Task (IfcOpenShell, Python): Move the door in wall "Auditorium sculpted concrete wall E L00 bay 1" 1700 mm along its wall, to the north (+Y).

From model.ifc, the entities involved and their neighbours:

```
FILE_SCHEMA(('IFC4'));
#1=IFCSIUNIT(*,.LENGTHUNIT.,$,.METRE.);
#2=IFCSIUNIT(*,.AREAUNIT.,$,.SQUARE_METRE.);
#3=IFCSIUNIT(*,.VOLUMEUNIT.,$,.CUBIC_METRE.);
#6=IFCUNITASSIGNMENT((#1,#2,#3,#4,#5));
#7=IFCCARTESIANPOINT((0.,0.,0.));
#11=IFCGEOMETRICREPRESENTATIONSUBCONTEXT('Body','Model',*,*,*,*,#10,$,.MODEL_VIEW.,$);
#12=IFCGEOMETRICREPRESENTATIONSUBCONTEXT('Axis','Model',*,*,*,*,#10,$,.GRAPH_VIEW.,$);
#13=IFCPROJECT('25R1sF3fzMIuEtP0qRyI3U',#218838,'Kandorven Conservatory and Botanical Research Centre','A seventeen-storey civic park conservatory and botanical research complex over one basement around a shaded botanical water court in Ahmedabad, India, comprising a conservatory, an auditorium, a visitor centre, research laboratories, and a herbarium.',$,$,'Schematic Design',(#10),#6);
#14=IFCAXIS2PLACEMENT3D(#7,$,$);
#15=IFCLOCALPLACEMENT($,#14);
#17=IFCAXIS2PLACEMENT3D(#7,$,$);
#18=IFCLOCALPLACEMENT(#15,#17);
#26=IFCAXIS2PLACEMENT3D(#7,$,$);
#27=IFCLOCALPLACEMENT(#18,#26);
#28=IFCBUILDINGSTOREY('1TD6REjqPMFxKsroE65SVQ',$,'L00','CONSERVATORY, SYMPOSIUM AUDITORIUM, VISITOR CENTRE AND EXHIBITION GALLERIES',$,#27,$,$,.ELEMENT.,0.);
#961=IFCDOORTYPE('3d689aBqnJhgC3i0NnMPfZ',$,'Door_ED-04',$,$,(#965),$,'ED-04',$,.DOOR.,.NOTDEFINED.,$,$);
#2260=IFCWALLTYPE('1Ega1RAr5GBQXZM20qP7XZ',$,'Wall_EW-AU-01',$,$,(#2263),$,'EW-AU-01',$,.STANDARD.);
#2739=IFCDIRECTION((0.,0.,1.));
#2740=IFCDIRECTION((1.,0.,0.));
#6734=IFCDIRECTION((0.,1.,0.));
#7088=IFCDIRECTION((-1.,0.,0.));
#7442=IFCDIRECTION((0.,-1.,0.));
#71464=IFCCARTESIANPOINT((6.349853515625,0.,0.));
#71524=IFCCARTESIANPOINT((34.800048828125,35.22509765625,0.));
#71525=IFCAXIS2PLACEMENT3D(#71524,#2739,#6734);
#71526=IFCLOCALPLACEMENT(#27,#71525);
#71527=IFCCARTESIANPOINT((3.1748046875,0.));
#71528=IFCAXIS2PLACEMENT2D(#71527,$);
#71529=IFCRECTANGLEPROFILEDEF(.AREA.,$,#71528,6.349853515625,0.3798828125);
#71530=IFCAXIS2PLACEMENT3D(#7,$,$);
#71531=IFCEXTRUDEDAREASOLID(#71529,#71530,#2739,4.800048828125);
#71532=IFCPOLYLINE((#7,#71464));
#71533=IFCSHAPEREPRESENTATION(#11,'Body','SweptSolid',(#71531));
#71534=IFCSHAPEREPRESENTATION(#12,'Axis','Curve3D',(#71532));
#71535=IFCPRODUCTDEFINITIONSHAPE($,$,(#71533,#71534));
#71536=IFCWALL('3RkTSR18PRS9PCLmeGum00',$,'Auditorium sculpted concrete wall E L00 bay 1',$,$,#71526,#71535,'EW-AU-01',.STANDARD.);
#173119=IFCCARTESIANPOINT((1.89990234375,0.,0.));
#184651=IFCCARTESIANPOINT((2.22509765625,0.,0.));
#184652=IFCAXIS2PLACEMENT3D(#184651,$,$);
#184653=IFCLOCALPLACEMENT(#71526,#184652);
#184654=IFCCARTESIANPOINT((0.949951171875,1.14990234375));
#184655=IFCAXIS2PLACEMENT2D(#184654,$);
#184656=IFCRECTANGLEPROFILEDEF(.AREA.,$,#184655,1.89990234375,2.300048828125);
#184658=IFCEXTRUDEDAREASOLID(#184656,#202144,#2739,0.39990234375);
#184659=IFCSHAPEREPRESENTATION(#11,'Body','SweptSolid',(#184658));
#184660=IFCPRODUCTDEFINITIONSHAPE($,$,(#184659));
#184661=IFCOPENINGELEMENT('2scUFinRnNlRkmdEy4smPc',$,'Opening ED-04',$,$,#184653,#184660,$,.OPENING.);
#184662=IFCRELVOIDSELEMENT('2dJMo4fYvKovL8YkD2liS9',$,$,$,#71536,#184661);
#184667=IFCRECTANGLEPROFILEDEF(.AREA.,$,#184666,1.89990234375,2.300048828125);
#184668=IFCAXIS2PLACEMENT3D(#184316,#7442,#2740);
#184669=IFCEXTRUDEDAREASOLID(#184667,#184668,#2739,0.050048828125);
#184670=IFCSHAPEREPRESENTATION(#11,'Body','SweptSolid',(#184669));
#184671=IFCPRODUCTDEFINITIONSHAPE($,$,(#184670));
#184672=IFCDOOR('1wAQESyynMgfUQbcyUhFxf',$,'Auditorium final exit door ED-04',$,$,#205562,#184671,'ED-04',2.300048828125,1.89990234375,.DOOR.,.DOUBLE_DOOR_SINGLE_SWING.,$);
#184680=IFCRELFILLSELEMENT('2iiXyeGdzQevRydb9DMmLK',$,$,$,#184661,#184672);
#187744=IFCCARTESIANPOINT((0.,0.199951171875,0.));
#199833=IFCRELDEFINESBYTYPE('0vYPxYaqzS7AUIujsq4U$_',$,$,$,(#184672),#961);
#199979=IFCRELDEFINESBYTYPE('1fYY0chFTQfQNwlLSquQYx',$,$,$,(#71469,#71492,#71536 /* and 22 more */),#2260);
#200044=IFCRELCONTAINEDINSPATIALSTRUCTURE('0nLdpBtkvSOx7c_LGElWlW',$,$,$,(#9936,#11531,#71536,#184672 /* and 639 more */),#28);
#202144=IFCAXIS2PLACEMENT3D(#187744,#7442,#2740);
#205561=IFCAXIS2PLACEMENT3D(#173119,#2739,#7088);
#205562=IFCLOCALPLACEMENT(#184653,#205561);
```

```python
import ifcopenshell
import ifcopenshell.api.geometry
import ifcopenshell.util.placement
import ifcopenshell.util.unit

model = ifcopenshell.open("model.ifc")
unit_scale = ifcopenshell.util.unit.calculate_unit_scale(model)

door = model.by_guid("1wAQESyynMgfUQbcyUhFxf")
opening = door.FillsVoids[0].RelatingOpeningElement
wall = opening.VoidsElements[0].RelatingBuildingElement

wall_matrix = ifcopenshell.util.placement.get_local_placement(wall.ObjectPlacement)
shift = wall_matrix[:3, 0] * 1.7 / unit_scale
before = ifcopenshell.util.placement.get_local_placement(door.ObjectPlacement)[:3, 3].copy()

# The door is placed relative to its opening, so it follows when the opening moves.
matrix = ifcopenshell.util.placement.get_local_placement(opening.ObjectPlacement)
matrix[:3, 3] += shift
ifcopenshell.api.geometry.edit_object_placement(
    model, product=opening, matrix=matrix, is_si=False, should_transform_children=True
)

after = ifcopenshell.util.placement.get_local_placement(door.ObjectPlacement)[:3, 3]
print("door moved by", (after - before).round(3) + 0.0)

model.write("model_edited.ifc")
```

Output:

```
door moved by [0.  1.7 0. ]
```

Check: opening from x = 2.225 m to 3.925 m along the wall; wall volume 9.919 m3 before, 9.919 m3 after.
